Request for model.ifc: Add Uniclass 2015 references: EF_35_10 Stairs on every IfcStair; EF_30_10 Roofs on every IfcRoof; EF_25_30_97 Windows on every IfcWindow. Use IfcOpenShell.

First a look at what the model holds.

```python
import ifcopenshell

model = ifcopenshell.open("model.ifc")
print(model.schema)
print("classifications:", [c.Name for c in model.by_type("IfcClassification")])
for ifc_class in ("IfcDoor", "IfcRoof", "IfcStair", "IfcWall", "IfcWindow"):
    print(ifc_class, len(model.by_type(ifc_class)))
```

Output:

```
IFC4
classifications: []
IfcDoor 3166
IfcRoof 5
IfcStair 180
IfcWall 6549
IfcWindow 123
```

```python
import ifcopenshell
import ifcopenshell.api.classification

model = ifcopenshell.open("model.ifc")

system = ifcopenshell.api.classification.add_classification(model, classification="Uniclass 2015")

codes = {
    "IfcStair": ("EF_35_10", "Stairs"),
    "IfcRoof": ("EF_30_10", "Roofs"),
    "IfcWindow": ("EF_25_30_97", "Windows"),
}
for ifc_class, (code, name) in codes.items():
    products = model.by_type(ifc_class)
    ifcopenshell.api.classification.add_reference(
        model, products=products, classification=system, identification=code, name=name
    )
    print(code, len(products))

model.write("model-out.ifc")
```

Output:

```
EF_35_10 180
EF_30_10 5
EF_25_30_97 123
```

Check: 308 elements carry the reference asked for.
